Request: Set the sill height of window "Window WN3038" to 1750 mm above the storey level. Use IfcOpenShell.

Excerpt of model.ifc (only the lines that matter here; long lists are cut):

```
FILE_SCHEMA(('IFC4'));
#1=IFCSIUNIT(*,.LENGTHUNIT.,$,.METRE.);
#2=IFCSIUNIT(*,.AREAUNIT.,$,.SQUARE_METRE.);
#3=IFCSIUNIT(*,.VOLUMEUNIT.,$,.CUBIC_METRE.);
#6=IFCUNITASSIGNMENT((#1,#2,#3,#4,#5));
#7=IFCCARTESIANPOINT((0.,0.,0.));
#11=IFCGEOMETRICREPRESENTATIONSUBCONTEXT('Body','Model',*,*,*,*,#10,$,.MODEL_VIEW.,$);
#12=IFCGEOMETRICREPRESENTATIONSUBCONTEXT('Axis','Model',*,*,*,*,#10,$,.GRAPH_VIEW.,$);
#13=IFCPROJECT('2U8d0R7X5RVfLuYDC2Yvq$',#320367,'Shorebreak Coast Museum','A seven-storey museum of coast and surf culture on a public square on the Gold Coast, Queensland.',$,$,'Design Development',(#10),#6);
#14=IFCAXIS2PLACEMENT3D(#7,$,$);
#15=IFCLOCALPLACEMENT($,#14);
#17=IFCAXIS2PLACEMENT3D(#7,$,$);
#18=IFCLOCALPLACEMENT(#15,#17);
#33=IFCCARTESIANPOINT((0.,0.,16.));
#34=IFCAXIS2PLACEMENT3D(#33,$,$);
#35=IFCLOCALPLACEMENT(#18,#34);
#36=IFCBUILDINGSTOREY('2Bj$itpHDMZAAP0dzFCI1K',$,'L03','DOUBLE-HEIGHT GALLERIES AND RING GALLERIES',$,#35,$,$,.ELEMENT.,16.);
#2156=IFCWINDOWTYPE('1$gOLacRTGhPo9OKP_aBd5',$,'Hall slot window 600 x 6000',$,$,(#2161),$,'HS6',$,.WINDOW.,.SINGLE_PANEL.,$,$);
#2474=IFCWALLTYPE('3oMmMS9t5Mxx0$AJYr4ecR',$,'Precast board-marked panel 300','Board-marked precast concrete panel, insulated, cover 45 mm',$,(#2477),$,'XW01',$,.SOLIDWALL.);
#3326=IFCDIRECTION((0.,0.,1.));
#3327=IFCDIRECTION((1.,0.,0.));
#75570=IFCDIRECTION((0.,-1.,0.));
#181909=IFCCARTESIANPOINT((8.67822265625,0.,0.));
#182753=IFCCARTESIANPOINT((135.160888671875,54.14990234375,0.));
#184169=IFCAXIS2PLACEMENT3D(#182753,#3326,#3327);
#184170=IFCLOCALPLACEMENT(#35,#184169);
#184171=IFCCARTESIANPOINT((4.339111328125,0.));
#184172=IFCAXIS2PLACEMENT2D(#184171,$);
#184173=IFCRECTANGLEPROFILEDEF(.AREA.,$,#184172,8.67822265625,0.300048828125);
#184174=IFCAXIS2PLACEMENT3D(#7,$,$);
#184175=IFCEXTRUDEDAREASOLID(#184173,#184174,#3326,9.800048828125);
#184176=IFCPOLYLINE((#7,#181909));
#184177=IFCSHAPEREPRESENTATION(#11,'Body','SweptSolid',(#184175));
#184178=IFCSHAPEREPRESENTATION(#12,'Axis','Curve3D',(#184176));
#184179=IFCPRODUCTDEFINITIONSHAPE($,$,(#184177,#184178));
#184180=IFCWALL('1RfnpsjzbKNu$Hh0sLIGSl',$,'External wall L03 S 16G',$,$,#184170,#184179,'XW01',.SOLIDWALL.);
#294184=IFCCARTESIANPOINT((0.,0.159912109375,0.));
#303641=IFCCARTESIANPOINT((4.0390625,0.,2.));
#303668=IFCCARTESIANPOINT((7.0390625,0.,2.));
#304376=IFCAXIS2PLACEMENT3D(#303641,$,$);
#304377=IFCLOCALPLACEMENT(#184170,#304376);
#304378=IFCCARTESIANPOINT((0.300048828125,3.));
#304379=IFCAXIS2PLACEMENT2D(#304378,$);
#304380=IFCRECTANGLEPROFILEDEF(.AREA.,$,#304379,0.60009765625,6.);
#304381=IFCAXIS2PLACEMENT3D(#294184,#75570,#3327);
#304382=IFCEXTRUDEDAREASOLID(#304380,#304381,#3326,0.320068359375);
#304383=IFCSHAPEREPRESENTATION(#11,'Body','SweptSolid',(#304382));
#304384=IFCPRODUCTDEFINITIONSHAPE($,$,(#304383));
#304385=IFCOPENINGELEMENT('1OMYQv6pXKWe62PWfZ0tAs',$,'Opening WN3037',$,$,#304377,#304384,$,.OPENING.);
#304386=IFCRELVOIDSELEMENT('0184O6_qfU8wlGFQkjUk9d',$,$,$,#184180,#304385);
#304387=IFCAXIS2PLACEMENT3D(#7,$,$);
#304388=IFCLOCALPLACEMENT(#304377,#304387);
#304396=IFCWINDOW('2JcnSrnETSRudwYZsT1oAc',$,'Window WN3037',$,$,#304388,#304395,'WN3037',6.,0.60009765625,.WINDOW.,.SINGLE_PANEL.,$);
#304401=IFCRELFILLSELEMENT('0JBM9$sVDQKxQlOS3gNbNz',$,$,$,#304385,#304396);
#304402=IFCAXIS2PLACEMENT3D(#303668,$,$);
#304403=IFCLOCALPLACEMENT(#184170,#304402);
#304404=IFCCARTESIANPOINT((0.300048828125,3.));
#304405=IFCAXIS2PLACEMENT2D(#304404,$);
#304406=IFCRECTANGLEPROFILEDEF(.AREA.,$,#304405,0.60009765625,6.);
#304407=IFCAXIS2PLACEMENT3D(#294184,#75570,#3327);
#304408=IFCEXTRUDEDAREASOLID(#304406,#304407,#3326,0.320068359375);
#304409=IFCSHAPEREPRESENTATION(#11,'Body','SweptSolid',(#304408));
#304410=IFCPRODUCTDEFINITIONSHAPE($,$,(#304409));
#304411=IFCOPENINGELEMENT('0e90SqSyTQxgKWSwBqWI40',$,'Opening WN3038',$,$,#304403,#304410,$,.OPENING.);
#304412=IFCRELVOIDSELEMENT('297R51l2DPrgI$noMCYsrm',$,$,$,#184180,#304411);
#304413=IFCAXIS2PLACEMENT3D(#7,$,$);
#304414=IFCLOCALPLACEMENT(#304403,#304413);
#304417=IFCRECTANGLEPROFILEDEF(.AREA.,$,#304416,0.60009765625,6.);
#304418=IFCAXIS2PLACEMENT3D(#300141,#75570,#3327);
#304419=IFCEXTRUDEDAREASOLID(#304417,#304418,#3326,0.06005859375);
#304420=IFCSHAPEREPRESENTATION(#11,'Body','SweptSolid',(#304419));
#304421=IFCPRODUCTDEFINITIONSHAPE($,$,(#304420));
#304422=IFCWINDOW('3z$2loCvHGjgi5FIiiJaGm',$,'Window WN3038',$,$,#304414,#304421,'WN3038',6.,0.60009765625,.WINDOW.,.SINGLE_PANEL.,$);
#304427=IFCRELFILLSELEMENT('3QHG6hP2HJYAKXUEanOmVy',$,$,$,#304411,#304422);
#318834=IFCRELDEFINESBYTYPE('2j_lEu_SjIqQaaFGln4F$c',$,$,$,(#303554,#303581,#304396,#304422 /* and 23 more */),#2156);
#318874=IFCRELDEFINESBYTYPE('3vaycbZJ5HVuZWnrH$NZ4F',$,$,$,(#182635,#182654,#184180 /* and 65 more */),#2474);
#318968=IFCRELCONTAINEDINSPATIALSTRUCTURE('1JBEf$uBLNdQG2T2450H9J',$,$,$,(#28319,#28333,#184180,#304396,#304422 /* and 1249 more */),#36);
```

```python
import numpy as np
import ifcopenshell
import ifcopenshell.api.geometry
import ifcopenshell.geom
import ifcopenshell.util.element
import ifcopenshell.util.placement
import ifcopenshell.util.shape
import ifcopenshell.util.unit

model = ifcopenshell.open("model.ifc")
unit_scale = ifcopenshell.util.unit.calculate_unit_scale(model)

window = model.by_id(304422)
opening = window.FillsVoids[0].RelatingOpeningElement
storey = ifcopenshell.util.element.get_container(window, ifc_class="IfcBuildingStorey")
level = ifcopenshell.util.placement.get_local_placement(storey.ObjectPlacement)[2, 3]

# The opening's origin need not be at the sill, so measure its lowest point.
shape = ifcopenshell.geom.create_shape(ifcopenshell.geom.settings(), opening)
bottom = ifcopenshell.util.shape.get_shape_bottom_elevation(shape, shape.geometry) / unit_scale
dz = level + 1.75 - bottom

shift = np.array([0.0, 0.0, dz])
# The window is placed relative to its opening, so it follows when the opening moves.
matrix = ifcopenshell.util.placement.get_local_placement(opening.ObjectPlacement)
matrix[:3, 3] += shift
ifcopenshell.api.geometry.edit_object_placement(
    model, product=opening, matrix=matrix, is_si=False, should_transform_children=True
)

print(f"moved by {dz * unit_scale:+.3f} m")

model.write("model_v2.ifc")
```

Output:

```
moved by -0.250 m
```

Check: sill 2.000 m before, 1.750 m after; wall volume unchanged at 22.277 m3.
